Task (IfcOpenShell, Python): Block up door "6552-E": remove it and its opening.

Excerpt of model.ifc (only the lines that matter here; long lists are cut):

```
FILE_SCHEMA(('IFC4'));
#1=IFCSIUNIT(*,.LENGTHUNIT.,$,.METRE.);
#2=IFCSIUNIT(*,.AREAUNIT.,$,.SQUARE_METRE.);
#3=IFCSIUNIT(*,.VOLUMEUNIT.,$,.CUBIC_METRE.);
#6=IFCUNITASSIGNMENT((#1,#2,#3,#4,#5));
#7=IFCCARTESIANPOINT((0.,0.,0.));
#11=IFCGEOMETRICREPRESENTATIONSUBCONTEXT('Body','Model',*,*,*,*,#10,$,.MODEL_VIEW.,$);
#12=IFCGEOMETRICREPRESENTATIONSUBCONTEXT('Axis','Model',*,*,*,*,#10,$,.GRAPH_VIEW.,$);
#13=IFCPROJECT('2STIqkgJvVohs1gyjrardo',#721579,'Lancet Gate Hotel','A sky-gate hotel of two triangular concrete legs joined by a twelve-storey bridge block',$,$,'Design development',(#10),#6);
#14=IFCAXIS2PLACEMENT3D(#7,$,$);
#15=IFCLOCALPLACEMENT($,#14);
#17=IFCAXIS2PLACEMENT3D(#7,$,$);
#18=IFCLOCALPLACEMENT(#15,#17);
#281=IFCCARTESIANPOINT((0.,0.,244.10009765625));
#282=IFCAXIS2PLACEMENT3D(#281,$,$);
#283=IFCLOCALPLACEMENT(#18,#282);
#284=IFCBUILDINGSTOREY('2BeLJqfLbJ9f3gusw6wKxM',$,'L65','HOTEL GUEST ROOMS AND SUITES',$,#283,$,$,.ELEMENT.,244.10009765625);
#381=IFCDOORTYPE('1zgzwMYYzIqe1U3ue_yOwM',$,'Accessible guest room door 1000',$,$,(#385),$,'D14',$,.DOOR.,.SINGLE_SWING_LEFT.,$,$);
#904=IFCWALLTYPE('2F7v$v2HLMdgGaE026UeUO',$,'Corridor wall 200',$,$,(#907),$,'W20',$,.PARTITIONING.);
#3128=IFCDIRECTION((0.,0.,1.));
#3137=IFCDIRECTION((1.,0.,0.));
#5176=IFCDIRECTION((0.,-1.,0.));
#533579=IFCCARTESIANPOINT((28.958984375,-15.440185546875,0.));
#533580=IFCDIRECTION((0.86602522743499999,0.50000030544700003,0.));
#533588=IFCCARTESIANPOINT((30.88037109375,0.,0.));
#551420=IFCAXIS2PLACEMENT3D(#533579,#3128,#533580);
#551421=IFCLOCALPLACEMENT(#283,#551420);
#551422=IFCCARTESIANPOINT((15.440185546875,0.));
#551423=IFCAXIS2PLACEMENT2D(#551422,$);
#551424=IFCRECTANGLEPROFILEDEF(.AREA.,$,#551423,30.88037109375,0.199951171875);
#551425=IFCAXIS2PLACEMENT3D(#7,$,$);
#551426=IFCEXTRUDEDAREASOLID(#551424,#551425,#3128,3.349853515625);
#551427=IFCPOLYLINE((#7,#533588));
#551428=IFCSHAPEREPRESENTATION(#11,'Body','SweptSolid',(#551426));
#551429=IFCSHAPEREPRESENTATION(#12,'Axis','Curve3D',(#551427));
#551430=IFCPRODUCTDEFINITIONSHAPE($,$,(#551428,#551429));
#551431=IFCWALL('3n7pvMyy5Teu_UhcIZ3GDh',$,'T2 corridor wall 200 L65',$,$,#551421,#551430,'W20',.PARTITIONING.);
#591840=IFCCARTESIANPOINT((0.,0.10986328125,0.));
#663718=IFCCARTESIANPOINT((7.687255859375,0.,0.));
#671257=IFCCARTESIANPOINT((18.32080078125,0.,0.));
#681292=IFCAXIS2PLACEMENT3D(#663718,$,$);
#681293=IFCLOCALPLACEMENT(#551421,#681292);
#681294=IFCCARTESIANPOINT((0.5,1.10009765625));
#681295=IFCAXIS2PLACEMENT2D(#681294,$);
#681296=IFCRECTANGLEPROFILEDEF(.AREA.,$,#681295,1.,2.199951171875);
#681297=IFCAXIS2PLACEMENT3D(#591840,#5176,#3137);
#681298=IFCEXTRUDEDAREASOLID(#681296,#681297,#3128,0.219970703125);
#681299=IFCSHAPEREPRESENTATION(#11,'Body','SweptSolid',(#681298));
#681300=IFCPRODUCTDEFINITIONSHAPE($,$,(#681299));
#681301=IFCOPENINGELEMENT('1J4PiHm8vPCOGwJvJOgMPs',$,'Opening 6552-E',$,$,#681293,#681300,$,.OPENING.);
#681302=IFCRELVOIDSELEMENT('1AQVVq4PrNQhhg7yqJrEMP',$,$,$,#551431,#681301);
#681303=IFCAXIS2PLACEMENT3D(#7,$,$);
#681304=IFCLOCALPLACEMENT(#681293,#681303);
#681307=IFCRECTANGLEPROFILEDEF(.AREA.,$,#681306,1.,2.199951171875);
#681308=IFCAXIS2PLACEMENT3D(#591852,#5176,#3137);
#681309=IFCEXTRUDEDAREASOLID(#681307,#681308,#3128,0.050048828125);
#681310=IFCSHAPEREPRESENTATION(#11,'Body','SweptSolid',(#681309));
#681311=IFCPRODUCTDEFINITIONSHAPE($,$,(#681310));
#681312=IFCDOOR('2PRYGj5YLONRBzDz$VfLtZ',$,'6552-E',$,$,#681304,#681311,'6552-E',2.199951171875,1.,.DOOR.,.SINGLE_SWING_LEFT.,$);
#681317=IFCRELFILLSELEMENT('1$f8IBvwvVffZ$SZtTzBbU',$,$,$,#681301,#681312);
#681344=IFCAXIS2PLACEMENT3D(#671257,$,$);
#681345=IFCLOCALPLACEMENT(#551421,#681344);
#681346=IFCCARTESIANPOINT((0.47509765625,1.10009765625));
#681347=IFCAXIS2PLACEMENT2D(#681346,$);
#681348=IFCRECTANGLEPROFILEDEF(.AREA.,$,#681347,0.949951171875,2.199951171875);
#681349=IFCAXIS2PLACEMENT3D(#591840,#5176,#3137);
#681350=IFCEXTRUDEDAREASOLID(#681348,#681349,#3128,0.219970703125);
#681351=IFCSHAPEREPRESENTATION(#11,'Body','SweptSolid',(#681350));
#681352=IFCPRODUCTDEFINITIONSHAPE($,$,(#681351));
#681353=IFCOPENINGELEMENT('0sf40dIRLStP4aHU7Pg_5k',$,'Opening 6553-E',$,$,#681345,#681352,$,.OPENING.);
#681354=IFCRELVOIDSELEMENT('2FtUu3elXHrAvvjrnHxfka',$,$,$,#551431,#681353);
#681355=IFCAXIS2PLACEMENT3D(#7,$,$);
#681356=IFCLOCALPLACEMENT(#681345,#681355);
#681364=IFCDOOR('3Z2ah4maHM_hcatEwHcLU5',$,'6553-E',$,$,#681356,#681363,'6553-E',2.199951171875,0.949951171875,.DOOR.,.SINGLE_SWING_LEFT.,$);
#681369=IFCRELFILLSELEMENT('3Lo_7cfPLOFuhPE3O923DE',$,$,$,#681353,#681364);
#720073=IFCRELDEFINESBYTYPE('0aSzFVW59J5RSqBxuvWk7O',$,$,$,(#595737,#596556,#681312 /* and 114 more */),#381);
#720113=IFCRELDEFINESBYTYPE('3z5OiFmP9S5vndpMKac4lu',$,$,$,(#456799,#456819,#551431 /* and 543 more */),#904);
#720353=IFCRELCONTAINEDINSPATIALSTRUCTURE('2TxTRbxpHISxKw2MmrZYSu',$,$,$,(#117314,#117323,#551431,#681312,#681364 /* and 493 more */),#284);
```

```python
import ifcopenshell
import ifcopenshell.api.feature
import ifcopenshell.api.root
import ifcopenshell.geom
import ifcopenshell.util.shape

model = ifcopenshell.open("model.ifc")
settings = ifcopenshell.geom.settings()


def volume(element):
    """Net volume in cubic metres, openings subtracted."""
    shape = ifcopenshell.geom.create_shape(settings, element)
    return ifcopenshell.util.shape.get_volume(shape.geometry)


door = model.by_id(681312)
opening = door.FillsVoids[0].RelatingOpeningElement
wall = opening.VoidsElements[0].RelatingBuildingElement
before = volume(wall)

ifcopenshell.api.root.remove_product(model, product=door)
ifcopenshell.api.feature.remove_feature(model, feature=opening)

after = volume(wall)

print(f"wall volume {before:.3f} -> {after:.3f} m3")

model.write("model_updated.ifc")
```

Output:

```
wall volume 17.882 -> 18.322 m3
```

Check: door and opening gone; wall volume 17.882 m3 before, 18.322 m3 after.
